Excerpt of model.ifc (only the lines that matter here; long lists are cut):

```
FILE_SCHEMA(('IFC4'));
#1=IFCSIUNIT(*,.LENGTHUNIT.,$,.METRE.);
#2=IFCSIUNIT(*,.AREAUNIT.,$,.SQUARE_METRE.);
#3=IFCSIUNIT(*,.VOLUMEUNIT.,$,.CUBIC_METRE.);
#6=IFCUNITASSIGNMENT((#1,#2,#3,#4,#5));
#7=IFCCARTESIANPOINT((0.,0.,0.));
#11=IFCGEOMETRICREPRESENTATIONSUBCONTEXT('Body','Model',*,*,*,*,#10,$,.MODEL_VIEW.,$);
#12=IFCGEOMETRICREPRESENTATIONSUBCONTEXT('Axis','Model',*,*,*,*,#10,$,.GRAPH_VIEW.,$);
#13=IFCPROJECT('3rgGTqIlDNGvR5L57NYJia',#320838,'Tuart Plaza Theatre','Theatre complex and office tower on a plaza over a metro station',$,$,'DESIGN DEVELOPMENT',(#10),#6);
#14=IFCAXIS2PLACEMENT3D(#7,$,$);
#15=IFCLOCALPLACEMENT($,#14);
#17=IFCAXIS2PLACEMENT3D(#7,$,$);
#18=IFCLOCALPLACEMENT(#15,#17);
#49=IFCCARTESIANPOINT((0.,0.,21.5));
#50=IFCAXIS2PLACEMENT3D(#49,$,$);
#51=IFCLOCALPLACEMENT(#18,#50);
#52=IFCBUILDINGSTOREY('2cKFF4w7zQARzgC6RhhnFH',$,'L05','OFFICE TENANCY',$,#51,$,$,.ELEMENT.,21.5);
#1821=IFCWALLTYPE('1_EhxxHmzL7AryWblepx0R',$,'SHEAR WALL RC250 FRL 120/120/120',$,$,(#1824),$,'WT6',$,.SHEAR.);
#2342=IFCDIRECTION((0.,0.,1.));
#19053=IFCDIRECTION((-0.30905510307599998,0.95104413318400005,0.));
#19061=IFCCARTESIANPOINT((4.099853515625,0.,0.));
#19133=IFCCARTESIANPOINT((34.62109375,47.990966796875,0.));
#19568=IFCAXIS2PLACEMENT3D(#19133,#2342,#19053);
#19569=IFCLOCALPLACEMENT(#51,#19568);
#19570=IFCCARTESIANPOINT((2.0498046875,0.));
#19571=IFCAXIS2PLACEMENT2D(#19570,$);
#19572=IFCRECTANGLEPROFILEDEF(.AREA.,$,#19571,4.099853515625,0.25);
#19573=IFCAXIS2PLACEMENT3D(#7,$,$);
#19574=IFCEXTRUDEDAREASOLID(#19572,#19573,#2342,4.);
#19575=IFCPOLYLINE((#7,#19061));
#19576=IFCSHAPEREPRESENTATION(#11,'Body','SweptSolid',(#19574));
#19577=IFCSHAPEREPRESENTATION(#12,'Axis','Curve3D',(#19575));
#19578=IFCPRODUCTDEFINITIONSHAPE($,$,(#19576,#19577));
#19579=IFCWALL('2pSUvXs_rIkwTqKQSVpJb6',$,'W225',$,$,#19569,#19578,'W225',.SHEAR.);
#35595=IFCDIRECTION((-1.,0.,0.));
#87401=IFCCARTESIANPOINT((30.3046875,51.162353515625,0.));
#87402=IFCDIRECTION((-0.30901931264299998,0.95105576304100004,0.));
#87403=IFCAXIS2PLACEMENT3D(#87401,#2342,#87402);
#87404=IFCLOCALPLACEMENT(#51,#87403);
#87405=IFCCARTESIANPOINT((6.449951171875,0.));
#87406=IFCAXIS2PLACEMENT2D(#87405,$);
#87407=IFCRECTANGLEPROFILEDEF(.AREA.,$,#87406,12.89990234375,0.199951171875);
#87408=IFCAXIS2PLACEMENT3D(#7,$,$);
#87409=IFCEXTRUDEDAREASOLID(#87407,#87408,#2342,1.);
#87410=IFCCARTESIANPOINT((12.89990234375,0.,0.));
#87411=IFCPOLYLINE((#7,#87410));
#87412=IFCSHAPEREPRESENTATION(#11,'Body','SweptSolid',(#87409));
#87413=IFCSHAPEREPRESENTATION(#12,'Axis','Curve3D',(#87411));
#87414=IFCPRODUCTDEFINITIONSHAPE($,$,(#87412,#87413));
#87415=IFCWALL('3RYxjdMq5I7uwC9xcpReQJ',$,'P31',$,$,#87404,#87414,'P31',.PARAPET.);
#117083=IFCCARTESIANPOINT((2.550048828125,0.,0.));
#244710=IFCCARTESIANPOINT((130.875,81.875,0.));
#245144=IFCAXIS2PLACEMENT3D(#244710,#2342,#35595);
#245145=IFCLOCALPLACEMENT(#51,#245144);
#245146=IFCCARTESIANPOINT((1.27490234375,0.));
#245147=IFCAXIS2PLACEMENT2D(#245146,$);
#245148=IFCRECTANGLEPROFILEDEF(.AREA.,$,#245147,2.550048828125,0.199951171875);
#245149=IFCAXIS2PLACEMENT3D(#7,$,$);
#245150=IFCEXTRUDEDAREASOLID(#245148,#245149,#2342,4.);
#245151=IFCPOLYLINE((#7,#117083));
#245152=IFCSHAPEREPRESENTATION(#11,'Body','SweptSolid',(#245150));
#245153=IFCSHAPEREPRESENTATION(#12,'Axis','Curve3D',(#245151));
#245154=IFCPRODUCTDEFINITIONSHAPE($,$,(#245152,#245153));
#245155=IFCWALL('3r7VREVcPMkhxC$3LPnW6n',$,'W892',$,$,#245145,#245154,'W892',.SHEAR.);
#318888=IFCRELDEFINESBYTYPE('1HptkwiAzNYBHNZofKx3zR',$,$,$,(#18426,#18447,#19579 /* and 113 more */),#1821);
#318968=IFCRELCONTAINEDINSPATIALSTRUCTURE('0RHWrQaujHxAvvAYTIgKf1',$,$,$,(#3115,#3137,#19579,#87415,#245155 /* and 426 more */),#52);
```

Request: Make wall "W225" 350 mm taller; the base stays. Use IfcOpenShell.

```python
import ifcopenshell
import ifcopenshell.geom
import ifcopenshell.util.representation
import ifcopenshell.util.shape

model = ifcopenshell.open("model.ifc")
settings = ifcopenshell.geom.settings()


def volume(element):
    """Net volume in cubic metres, openings subtracted."""
    shape = ifcopenshell.geom.create_shape(settings, element)
    return ifcopenshell.util.shape.get_volume(shape.geometry)


wall = model.by_id(19579)
before = volume(wall)

body = ifcopenshell.util.representation.get_representation(wall, "Model", "Body")
solid = body.Items[0]
old_height = solid.Depth
solid.Depth += 0.35
after = volume(wall)

print(f"height {old_height:g} -> {solid.Depth:g}, volume {before:.3f} -> {after:.3f} m3")

model.write("model_rev.ifc")
```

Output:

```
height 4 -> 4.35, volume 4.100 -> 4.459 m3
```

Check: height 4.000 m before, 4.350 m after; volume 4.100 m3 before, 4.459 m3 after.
